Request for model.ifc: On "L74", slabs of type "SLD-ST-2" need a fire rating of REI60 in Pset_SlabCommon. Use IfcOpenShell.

First a look at what the model holds.

```python
import ifcopenshell
import ifcopenshell.util.element

model = ifcopenshell.open("model.ifc")
print(model.schema)
storey = next(s for s in model.by_type("IfcBuildingStorey") if s.Name == "L74")
slabs = [e for e in ifcopenshell.util.element.get_decomposition(storey) if e.is_a("IfcSlab")]
seen = {}
for e in slabs:
    element_type = ifcopenshell.util.element.get_type(e)
    key = (element_type.Name if element_type != e and element_type else None, ifcopenshell.util.element.get_pset(e, "Pset_SlabCommon", "FireRating"))
    seen[key] = seen.get(key, 0) + 1
for (name, value), count in sorted(seen.items(), key=str):
    print(count, "x", name, "|", value)
```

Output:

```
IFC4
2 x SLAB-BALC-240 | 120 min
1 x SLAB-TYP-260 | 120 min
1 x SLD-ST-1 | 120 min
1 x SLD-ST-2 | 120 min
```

```python
import ifcopenshell
import ifcopenshell.api.pset
import ifcopenshell.util.element

model = ifcopenshell.open("model.ifc")

storey = next(s for s in model.by_type("IfcBuildingStorey") if s.Name == "L74")
slabs = [e for e in ifcopenshell.util.element.get_decomposition(storey) if e.is_a("IfcSlab")]

count = 0
for e in slabs:
    element_type = ifcopenshell.util.element.get_type(e)
    if element_type in (None, e) or element_type.Name != "SLD-ST-2":
        continue
    found = ifcopenshell.util.element.get_pset(e, "Pset_SlabCommon", should_inherit=False)
    if found:
        pset = model.by_id(found["id"])
        if len(ifcopenshell.util.element.get_elements_by_pset(pset)) > 1:
            pset = ifcopenshell.api.pset.unshare_pset(model, products=[e], pset=pset)[0]
    else:
        pset = ifcopenshell.api.pset.add_pset(model, product=e, name="Pset_SlabCommon")
    ifcopenshell.api.pset.edit_pset(model, pset=pset, properties={"FireRating": "REI60"})
    count += 1

print(count, "slabs updated")

model.write("model_v2.ifc")
```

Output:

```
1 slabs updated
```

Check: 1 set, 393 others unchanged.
